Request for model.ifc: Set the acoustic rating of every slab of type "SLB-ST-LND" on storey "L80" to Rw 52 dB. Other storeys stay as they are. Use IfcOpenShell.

First a look at what the model holds.

```python
import ifcopenshell
import ifcopenshell.util.element

model = ifcopenshell.open("model.ifc")
print(model.schema)
storey = next(s for s in model.by_type("IfcBuildingStorey") if s.Name == "L80")
slabs = [e for e in ifcopenshell.util.element.get_decomposition(storey) if e.is_a("IfcSlab")]
seen = {}
for e in slabs:
    element_type = ifcopenshell.util.element.get_type(e)
    key = (element_type.Name if element_type != e and element_type else None, ifcopenshell.util.element.get_pset(e, "Pset_SlabCommon", "AcousticRating"))
    seen[key] = seen.get(key, 0) + 1
for (name, value), count in sorted(seen.items(), key=str):
    print(count, "x", name, "|", value)
```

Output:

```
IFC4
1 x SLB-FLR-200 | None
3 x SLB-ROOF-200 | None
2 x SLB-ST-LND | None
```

```python
import ifcopenshell
import ifcopenshell.api.pset
import ifcopenshell.util.element

model = ifcopenshell.open("model.ifc")

storey = next(s for s in model.by_type("IfcBuildingStorey") if s.Name == "L80")
slabs = [e for e in ifcopenshell.util.element.get_decomposition(storey) if e.is_a("IfcSlab")]

count = 0
for e in slabs:
    element_type = ifcopenshell.util.element.get_type(e)
    if element_type in (None, e) or element_type.Name != "SLB-ST-LND":
        continue
    found = ifcopenshell.util.element.get_pset(e, "Pset_SlabCommon", should_inherit=False)
    if found:
        pset = model.by_id(found["id"])
        if len(ifcopenshell.util.element.get_elements_by_pset(pset)) > 1:
            pset = ifcopenshell.api.pset.unshare_pset(model, products=[e], pset=pset)[0]
    else:
        pset = ifcopenshell.api.pset.add_pset(model, product=e, name="Pset_SlabCommon")
    ifcopenshell.api.pset.edit_pset(model, pset=pset, properties={"AcousticRating": "Rw 52 dB"})
    count += 1

print(count, "slabs updated")

model.write("model_edited.ifc")
```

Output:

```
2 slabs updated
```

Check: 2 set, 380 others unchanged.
